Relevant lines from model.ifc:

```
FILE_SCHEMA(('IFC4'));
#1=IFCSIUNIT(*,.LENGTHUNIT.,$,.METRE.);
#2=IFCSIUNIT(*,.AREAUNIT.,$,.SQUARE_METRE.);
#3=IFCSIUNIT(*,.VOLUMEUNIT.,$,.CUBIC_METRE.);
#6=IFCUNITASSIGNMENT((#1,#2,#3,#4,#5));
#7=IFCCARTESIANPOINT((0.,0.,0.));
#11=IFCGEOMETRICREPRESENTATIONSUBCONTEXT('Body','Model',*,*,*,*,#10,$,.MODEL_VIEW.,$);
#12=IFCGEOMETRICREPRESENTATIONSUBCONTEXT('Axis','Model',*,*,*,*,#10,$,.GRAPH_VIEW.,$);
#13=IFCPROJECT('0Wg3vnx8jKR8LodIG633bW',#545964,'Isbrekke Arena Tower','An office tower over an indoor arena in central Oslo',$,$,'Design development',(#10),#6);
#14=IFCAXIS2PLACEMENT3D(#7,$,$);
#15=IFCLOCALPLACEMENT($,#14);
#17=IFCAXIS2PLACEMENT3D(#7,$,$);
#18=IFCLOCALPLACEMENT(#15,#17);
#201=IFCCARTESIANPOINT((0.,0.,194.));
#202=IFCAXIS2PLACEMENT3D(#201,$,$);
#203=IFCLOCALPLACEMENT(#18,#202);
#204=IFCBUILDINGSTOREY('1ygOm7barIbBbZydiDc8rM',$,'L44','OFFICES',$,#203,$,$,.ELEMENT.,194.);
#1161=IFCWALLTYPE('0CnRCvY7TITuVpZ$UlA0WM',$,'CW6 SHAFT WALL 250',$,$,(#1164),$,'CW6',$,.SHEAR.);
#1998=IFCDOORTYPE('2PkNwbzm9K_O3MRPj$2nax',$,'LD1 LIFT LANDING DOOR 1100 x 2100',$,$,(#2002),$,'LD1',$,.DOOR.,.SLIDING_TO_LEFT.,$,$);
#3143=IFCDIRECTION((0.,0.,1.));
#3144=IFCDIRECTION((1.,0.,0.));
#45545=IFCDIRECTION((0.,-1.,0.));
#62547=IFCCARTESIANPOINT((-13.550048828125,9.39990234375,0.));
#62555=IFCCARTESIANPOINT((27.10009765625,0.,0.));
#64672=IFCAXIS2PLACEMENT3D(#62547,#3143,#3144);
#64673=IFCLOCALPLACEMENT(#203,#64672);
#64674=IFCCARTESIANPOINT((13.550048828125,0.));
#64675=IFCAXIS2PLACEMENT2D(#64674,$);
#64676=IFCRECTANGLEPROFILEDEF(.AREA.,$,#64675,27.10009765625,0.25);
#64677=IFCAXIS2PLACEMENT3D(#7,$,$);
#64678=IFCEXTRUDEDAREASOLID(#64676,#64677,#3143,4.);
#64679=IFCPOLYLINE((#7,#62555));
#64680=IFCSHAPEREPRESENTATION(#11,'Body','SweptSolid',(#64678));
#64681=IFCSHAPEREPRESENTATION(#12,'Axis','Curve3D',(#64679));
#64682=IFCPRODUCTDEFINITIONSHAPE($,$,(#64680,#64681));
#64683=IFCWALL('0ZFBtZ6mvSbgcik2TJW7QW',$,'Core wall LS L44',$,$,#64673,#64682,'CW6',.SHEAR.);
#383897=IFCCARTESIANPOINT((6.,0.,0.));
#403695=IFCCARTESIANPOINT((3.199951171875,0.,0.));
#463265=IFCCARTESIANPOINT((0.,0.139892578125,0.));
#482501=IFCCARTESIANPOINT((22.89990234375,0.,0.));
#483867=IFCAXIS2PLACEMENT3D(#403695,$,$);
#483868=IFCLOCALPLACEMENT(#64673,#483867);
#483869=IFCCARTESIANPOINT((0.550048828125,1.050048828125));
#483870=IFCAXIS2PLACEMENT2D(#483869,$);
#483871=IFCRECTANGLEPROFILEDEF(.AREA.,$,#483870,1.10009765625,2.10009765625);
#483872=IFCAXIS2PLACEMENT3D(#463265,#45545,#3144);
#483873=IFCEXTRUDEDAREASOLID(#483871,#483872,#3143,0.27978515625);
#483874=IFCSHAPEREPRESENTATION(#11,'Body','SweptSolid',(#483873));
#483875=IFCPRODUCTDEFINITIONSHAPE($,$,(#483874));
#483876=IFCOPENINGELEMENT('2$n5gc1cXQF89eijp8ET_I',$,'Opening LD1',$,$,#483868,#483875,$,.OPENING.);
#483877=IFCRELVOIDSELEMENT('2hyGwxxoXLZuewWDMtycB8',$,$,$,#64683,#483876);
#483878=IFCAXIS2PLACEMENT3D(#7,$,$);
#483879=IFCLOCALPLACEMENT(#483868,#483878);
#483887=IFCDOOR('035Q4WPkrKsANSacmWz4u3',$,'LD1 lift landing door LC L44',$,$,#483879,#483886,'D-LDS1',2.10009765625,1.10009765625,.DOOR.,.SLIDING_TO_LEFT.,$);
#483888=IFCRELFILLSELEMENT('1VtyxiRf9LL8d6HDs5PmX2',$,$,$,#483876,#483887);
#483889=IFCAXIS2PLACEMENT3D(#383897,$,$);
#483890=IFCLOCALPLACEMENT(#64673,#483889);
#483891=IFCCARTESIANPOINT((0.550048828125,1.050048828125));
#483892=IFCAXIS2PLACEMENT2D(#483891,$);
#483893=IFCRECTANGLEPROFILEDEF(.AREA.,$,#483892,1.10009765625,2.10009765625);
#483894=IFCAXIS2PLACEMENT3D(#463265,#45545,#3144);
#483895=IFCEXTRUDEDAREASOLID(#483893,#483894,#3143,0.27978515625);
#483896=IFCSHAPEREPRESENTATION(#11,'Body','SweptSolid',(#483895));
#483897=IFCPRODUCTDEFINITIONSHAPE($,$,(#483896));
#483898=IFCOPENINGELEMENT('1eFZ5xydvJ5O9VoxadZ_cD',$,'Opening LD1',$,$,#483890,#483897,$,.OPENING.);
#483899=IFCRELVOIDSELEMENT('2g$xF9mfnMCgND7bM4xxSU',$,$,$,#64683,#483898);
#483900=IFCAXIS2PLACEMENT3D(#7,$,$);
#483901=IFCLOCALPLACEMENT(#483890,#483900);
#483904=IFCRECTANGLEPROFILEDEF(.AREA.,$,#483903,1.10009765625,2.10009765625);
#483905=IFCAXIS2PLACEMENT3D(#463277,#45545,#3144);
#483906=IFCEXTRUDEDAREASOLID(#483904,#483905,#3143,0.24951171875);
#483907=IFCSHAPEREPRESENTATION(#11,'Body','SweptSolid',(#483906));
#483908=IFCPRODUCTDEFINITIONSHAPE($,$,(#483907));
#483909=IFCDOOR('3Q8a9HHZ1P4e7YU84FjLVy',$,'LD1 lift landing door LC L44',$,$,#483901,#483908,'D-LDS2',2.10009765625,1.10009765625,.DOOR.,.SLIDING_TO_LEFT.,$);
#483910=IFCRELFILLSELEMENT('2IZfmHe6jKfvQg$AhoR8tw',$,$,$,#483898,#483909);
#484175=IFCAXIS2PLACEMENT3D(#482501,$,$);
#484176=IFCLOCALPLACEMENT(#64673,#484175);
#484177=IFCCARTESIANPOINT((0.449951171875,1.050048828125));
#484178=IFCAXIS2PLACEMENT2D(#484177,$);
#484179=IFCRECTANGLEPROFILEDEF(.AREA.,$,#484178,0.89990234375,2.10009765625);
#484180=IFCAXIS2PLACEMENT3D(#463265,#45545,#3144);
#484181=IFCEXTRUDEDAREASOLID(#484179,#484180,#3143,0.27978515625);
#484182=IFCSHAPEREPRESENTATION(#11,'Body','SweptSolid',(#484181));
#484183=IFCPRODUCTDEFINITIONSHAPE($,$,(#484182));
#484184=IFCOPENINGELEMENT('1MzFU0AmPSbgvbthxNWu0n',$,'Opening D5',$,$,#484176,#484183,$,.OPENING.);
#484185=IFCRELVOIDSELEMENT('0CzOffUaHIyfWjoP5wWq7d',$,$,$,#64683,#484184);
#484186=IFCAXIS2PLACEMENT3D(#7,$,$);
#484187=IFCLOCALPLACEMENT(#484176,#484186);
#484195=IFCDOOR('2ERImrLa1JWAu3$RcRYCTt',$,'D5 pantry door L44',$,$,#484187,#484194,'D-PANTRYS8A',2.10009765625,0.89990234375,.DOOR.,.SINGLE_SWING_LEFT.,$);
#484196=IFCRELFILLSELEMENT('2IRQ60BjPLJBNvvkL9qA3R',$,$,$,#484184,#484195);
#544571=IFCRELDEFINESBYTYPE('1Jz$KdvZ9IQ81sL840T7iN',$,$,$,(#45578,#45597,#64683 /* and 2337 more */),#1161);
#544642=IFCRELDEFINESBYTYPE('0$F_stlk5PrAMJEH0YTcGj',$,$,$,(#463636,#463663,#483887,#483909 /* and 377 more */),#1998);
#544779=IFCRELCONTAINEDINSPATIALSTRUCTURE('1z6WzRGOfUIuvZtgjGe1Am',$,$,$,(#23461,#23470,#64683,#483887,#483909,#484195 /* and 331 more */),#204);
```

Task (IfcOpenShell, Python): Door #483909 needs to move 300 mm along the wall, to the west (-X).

```python
import ifcopenshell
import ifcopenshell.api.geometry
import ifcopenshell.util.placement

model = ifcopenshell.open("model.ifc")

door = model.by_id(483909)
opening = door.FillsVoids[0].RelatingOpeningElement
wall = opening.VoidsElements[0].RelatingBuildingElement

wall_matrix = ifcopenshell.util.placement.get_local_placement(wall.ObjectPlacement)
shift = wall_matrix[:3, 0] * -0.3
before = ifcopenshell.util.placement.get_local_placement(door.ObjectPlacement)[:3, 3].copy()

# The door is placed relative to its opening, so it follows when the opening moves.
matrix = ifcopenshell.util.placement.get_local_placement(opening.ObjectPlacement)
matrix[:3, 3] += shift
ifcopenshell.api.geometry.edit_object_placement(
    model, product=opening, matrix=matrix, is_si=False, should_transform_children=True
)

after = ifcopenshell.util.placement.get_local_placement(door.ObjectPlacement)[:3, 3]
print("door moved by", (after - before).round(3) + 0.0)

model.write("model_updated.ifc")
```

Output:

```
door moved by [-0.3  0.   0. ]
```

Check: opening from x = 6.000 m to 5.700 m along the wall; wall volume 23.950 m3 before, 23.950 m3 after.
